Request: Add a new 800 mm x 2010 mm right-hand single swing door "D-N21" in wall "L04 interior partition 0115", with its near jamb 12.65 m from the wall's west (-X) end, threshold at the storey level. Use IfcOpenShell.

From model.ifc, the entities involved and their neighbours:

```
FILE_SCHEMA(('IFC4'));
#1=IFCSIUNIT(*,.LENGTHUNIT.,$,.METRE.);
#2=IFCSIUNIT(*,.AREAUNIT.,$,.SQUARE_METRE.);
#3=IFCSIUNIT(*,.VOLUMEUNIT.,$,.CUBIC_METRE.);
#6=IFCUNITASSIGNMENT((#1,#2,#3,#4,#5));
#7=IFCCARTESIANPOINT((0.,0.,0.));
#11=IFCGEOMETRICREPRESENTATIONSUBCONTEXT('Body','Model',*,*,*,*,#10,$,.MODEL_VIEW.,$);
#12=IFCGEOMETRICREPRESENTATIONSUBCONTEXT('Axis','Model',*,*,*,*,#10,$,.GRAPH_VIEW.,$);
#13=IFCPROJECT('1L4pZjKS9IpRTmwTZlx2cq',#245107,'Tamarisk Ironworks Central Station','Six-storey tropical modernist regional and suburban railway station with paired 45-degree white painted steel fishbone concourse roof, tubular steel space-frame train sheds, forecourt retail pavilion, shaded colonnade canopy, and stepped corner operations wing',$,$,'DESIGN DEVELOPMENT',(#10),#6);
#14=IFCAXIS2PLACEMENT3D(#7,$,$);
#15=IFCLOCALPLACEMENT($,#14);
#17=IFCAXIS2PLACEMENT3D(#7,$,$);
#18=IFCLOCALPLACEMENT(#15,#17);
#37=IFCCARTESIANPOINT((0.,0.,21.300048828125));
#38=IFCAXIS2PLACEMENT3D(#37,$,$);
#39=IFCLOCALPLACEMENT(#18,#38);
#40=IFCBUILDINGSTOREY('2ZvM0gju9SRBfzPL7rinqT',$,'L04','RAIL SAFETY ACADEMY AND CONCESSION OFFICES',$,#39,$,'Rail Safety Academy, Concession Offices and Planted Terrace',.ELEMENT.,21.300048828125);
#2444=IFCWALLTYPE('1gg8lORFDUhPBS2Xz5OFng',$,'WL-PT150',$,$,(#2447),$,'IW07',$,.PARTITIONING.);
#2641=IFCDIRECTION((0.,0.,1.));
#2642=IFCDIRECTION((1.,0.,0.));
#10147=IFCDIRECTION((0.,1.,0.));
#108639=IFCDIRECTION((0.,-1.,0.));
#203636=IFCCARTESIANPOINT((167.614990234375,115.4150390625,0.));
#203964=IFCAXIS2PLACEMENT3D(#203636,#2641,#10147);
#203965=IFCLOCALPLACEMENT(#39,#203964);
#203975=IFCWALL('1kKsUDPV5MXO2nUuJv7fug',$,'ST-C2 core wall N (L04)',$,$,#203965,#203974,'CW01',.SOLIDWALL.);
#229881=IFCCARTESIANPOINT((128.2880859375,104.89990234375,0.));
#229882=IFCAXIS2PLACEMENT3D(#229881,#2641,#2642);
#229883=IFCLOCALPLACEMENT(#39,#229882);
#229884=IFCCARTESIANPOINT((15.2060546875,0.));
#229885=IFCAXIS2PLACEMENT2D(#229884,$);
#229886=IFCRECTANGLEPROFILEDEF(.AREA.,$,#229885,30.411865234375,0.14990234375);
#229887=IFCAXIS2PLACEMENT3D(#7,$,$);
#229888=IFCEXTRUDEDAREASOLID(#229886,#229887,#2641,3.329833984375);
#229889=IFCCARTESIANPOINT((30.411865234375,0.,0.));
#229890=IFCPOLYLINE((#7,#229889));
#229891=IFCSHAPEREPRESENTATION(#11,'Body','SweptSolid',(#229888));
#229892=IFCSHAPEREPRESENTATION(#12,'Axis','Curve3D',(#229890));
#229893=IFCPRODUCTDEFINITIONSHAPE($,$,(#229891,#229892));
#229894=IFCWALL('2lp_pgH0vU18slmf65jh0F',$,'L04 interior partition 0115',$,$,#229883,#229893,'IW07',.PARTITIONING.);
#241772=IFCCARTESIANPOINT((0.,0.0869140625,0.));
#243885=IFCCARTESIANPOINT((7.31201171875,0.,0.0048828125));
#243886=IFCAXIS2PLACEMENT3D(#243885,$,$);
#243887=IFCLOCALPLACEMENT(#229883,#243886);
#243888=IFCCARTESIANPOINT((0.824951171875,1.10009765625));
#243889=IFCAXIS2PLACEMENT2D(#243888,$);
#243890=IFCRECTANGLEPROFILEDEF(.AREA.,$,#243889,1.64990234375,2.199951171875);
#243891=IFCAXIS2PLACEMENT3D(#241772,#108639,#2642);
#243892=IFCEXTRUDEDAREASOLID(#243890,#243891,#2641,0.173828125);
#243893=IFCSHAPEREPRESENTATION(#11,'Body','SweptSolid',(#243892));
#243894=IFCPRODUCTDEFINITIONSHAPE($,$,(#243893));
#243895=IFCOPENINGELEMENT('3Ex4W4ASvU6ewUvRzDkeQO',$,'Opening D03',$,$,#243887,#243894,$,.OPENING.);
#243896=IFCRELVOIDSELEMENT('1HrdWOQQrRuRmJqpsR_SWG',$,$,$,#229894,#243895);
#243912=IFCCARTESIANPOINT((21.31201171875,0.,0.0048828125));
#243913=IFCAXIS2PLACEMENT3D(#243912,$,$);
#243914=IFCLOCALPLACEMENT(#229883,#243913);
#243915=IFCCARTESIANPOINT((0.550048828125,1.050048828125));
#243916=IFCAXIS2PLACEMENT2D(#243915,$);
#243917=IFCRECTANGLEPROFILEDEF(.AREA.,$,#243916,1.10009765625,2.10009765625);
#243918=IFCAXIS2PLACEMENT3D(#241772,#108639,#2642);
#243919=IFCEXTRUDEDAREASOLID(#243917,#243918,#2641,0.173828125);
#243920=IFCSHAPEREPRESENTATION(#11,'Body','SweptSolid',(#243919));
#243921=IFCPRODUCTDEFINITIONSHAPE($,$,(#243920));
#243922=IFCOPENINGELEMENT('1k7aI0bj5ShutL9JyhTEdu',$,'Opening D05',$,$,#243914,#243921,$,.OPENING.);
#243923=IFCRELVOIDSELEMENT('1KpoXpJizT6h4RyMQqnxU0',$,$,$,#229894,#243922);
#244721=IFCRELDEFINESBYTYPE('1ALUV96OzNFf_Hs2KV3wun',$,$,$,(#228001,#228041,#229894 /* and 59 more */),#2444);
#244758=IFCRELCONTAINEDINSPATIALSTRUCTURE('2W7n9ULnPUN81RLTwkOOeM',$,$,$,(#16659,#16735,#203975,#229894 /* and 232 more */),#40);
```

```python
import numpy as np
import ifcopenshell
import ifcopenshell.api.feature
import ifcopenshell.api.geometry
import ifcopenshell.api.root
import ifcopenshell.api.spatial
import ifcopenshell.geom
import ifcopenshell.util.element
import ifcopenshell.util.placement
import ifcopenshell.util.representation
import ifcopenshell.util.shape
import ifcopenshell.util.unit

model = ifcopenshell.open("model.ifc")
unit_scale = ifcopenshell.util.unit.calculate_unit_scale(model)
settings = ifcopenshell.geom.settings()


def volume(element):
    """Net volume in cubic metres, openings subtracted."""
    shape = ifcopenshell.geom.create_shape(settings, element)
    return ifcopenshell.util.shape.get_volume(shape.geometry)


wall = model.by_guid("2lp_pgH0vU18slmf65jh0F")
storey = ifcopenshell.util.element.get_container(wall, ifc_class="IfcBuildingStorey")
context = ifcopenshell.util.representation.get_context(model, "Model", "Body", "MODEL_VIEW")
before = volume(wall)

width, height, from_end, sill = 0.8, 2.01, 12.65, 0.0  # metres

# The wall runs along its own X axis, and the end named is its -X end.
wall_shape = ifcopenshell.geom.create_shape(settings, wall)
x, y, z = ifcopenshell.util.shape.get_vertices(wall_shape.geometry).T
start = x.min() + from_end
face, thickness = float(y.min()), float(y.max() - y.min())
wall_matrix = ifcopenshell.util.placement.get_local_placement(wall.ObjectPlacement)
level = ifcopenshell.util.placement.get_local_placement(storey.ObjectPlacement)[2, 3]


def in_wall(x, y):
    """Placement at x, y metres in the wall's axes, at sill height."""
    matrix = wall_matrix.copy()
    matrix[:, 3] = wall_matrix @ np.array([x / unit_scale, y / unit_scale, 0.0, 1.0])
    matrix[2, 3] = level + sill / unit_scale
    return matrix


# Opening: a box that overshoots both wall faces by 50 mm.
opening = ifcopenshell.api.root.create_entity(model, ifc_class="IfcOpeningElement", predefined_type="OPENING")
box = ifcopenshell.api.geometry.add_wall_representation(
    model, context=context, length=width, height=height, thickness=thickness + 0.1
)
ifcopenshell.api.geometry.assign_representation(model, product=opening, representation=box)
ifcopenshell.api.geometry.edit_object_placement(model, product=opening, matrix=in_wall(start, face - 0.05), is_si=False)
ifcopenshell.api.feature.add_feature(model, feature=opening, element=wall)

door = ifcopenshell.api.root.create_entity(model, ifc_class="IfcDoor", name="D-N21", predefined_type="DOOR")
door.OverallWidth, door.OverallHeight = width / unit_scale, height / unit_scale
door.OperationType = "SINGLE_SWING_RIGHT"
body = ifcopenshell.api.geometry.add_door_representation(
    model,
    context=context,
    overall_width=door.OverallWidth,
    overall_height=door.OverallHeight,
    operation_type="SINGLE_SWING_RIGHT",
    lining_properties={"LiningDepth": thickness / unit_scale, "ThresholdDepth": thickness / unit_scale},
)
ifcopenshell.api.geometry.assign_representation(model, product=door, representation=body)
ifcopenshell.api.spatial.assign_container(model, products=[door], relating_structure=storey)
ifcopenshell.api.feature.add_filling(model, opening=opening, element=door)

# The lining spans the wall, so the door starts at the wall face.
ifcopenshell.api.geometry.edit_object_placement(model, product=door, matrix=in_wall(start, face), is_si=False)

after = volume(wall)

print(f"wall volume {before:.3f} -> {after:.3f} m3")

model.write("model-out.ifc")
```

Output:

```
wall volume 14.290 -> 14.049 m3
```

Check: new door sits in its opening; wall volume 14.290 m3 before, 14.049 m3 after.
